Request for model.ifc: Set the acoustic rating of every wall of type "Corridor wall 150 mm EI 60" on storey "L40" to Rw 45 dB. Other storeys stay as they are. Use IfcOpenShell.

First a look at what the model holds.

```python
import ifcopenshell
import ifcopenshell.util.element

model = ifcopenshell.open("model.ifc")
print(model.schema)
storey = next(s for s in model.by_type("IfcBuildingStorey") if s.Name == "L40")
walls = [e for e in ifcopenshell.util.element.get_decomposition(storey) if e.is_a("IfcWall")]
seen = {}
for e in walls:
    element_type = ifcopenshell.util.element.get_type(e)
    key = (element_type.Name if element_type != e and element_type else None, ifcopenshell.util.element.get_pset(e, "Pset_WallCommon", "AcousticRating"))
    seen[key] = seen.get(key, 0) + 1
for (name, value), count in sorted(seen.items(), key=str):
    print(count, "x", name, "|", value)
```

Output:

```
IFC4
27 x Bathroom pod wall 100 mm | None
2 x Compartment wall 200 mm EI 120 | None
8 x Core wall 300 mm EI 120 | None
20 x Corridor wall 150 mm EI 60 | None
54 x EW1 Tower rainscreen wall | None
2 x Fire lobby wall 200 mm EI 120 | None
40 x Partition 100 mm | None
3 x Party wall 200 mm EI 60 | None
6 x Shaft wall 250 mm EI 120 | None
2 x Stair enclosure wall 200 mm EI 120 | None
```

```python
import ifcopenshell
import ifcopenshell.api.pset
import ifcopenshell.util.element

model = ifcopenshell.open("model.ifc")

storey = next(s for s in model.by_type("IfcBuildingStorey") if s.Name == "L40")
walls = [e for e in ifcopenshell.util.element.get_decomposition(storey) if e.is_a("IfcWall")]

count = 0
for e in walls:
    element_type = ifcopenshell.util.element.get_type(e)
    if element_type in (None, e) or element_type.Name != "Corridor wall 150 mm EI 60":
        continue
    found = ifcopenshell.util.element.get_pset(e, "Pset_WallCommon", should_inherit=False)
    if found:
        pset = model.by_id(found["id"])
        if len(ifcopenshell.util.element.get_elements_by_pset(pset)) > 1:
            pset = ifcopenshell.api.pset.unshare_pset(model, products=[e], pset=pset)[0]
    else:
        pset = ifcopenshell.api.pset.add_pset(model, product=e, name="Pset_WallCommon")
    ifcopenshell.api.pset.edit_pset(model, pset=pset, properties={"AcousticRating": "Rw 45 dB"})
    count += 1

print(count, "walls updated")

model.write("model-out.ifc")
```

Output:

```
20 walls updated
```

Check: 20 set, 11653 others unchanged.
